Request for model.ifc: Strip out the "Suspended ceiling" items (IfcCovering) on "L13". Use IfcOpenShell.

First a look at what the model holds.

```python
import ifcopenshell
import ifcopenshell.util.element

model = ifcopenshell.open("model.ifc")
print(model.schema)
storey = next(s for s in model.by_type("IfcBuildingStorey") if s.Name == "L13")
coverings = [e for e in ifcopenshell.util.element.get_decomposition(storey) if e.is_a("IfcCovering")]
seen = {}
for e in coverings:
    element_type = ifcopenshell.util.element.get_type(e)
    name = element_type.Name if element_type not in (None, e) else None
    seen[name] = seen.get(name, 0) + 1
for name, count in sorted(seen.items(), key=str):
    print(count, "x", name)
```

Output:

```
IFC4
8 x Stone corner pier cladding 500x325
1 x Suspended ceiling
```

```python
import ifcopenshell
import ifcopenshell.api.root
import ifcopenshell.util.element

model = ifcopenshell.open("model.ifc")

storey = next(s for s in model.by_type("IfcBuildingStorey") if s.Name == "L13")
coverings = [e for e in ifcopenshell.util.element.get_decomposition(storey) if e.is_a("IfcCovering")]
targets = [e for e in coverings if (t := ifcopenshell.util.element.get_type(e)) not in (None, e) and t.Name == "Suspended ceiling"]

for e in targets:
    ifcopenshell.api.root.remove_product(model, product=e)
print(len(targets), "removed")

model.write("model_rev.ifc")
```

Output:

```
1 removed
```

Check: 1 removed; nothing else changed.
